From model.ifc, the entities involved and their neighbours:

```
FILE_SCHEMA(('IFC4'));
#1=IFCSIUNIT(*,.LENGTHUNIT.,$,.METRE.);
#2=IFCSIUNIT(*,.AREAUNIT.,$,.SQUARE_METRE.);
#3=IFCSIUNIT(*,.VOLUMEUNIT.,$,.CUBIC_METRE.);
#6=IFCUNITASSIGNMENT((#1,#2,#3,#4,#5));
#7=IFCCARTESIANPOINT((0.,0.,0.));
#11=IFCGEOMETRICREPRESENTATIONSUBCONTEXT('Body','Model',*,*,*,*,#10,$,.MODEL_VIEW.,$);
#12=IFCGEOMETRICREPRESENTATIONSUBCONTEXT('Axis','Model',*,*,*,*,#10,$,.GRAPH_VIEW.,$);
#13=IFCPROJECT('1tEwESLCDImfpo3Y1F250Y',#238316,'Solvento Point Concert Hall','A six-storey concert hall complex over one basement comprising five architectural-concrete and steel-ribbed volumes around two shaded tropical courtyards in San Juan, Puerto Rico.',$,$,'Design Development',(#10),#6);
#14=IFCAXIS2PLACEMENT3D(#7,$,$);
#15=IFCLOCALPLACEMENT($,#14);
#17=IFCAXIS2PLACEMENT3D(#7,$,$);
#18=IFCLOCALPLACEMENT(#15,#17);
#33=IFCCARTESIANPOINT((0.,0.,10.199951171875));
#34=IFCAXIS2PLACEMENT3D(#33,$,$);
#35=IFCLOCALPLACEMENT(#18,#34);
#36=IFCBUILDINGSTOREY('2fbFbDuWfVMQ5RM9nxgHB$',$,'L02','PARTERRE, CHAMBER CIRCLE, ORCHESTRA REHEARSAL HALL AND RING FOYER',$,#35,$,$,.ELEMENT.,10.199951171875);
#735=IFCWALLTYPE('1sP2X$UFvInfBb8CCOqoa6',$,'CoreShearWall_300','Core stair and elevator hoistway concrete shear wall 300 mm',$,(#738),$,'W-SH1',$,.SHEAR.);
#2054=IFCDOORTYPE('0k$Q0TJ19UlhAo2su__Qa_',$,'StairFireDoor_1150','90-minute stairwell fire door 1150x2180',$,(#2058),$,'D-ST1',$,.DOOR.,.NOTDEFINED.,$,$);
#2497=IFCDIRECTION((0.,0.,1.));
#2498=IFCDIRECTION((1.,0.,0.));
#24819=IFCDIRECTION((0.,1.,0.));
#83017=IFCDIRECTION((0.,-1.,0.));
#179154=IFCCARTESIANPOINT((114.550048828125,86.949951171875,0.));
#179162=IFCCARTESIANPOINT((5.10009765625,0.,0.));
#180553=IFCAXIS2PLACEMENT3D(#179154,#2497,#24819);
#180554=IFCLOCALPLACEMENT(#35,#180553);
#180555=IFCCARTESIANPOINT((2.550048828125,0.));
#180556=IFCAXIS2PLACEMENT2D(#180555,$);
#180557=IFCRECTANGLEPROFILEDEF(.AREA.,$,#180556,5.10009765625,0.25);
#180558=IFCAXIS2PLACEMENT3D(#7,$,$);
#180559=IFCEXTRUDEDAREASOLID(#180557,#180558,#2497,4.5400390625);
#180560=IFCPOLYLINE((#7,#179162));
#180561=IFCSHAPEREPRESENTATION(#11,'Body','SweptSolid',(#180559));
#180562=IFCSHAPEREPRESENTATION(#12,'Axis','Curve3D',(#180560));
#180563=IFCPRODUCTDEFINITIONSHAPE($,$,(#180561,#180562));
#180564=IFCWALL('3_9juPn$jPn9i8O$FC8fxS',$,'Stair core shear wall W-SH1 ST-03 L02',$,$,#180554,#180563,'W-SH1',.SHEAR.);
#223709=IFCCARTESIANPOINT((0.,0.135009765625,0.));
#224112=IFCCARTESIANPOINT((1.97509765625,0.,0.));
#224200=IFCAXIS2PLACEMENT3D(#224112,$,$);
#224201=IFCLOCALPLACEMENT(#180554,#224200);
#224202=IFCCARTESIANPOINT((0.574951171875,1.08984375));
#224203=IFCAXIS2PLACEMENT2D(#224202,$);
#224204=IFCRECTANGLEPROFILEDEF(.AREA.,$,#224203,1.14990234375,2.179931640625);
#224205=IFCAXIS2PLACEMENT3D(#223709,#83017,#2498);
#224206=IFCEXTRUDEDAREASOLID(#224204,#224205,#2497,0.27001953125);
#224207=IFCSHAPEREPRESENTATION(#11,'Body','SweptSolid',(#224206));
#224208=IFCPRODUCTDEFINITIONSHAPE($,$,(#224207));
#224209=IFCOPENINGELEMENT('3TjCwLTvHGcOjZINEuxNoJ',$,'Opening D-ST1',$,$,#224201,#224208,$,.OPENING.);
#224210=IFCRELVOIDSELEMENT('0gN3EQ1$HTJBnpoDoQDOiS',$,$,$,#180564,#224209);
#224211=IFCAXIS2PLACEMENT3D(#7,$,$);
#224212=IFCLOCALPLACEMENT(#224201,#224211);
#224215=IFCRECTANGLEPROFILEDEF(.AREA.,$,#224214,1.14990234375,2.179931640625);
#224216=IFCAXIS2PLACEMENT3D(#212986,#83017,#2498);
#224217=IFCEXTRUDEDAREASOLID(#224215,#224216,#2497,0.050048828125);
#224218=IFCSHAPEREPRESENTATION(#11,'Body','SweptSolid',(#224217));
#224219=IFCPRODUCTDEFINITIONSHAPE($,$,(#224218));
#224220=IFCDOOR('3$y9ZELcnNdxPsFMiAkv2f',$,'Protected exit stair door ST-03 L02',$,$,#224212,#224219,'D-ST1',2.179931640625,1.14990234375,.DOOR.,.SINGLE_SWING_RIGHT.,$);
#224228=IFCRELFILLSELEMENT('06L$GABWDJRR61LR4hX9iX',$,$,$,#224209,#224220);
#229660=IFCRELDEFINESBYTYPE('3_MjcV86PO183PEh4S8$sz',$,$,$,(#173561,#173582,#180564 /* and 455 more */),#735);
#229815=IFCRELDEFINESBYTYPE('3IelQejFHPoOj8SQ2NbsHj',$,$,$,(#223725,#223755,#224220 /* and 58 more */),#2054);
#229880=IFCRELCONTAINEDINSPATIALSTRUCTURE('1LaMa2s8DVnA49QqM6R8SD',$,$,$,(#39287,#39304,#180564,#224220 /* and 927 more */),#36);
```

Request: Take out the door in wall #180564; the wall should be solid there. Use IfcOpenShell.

```python
import ifcopenshell
import ifcopenshell.api.feature
import ifcopenshell.api.root
import ifcopenshell.geom
import ifcopenshell.util.shape

model = ifcopenshell.open("model.ifc")
settings = ifcopenshell.geom.settings()


def volume(element):
    """Net volume in cubic metres, openings subtracted."""
    shape = ifcopenshell.geom.create_shape(settings, element)
    return ifcopenshell.util.shape.get_volume(shape.geometry)


door = model.by_guid("3$y9ZELcnNdxPsFMiAkv2f")
opening = door.FillsVoids[0].RelatingOpeningElement
wall = opening.VoidsElements[0].RelatingBuildingElement
before = volume(wall)

ifcopenshell.api.root.remove_product(model, product=door)
ifcopenshell.api.feature.remove_feature(model, feature=opening)

after = volume(wall)

print(f"wall volume {before:.3f} -> {after:.3f} m3")

model.write("model_edited.ifc")
```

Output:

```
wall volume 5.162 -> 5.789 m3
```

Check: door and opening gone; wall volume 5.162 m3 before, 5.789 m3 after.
